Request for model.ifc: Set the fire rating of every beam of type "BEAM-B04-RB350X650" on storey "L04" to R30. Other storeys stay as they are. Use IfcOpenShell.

First a look at what the model holds.

```python
import ifcopenshell
import ifcopenshell.util.element

model = ifcopenshell.open("model.ifc")
print(model.schema)
storey = next(s for s in model.by_type("IfcBuildingStorey") if s.Name == "L04")
beams = [e for e in ifcopenshell.util.element.get_decomposition(storey) if e.is_a("IfcBeam")]
seen = {}
for e in beams:
    element_type = ifcopenshell.util.element.get_type(e)
    key = (element_type.Name if element_type != e and element_type else None, ifcopenshell.util.element.get_pset(e, "Pset_BeamCommon", "FireRating"))
    seen[key] = seen.get(key, 0) + 1
for (name, value), count in sorted(seen.items(), key=str):
    print(count, "x", name, "|", value)
```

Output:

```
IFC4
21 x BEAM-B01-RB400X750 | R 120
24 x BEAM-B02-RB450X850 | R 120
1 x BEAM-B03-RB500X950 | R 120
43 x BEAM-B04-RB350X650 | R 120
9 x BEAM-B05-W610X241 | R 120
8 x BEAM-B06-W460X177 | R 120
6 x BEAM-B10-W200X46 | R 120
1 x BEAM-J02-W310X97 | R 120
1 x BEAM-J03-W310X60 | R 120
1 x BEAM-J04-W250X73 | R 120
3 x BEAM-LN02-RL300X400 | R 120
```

```python
import ifcopenshell
import ifcopenshell.api.pset
import ifcopenshell.util.element

model = ifcopenshell.open("model.ifc")

storey = next(s for s in model.by_type("IfcBuildingStorey") if s.Name == "L04")
beams = [e for e in ifcopenshell.util.element.get_decomposition(storey) if e.is_a("IfcBeam")]

count = 0
for e in beams:
    element_type = ifcopenshell.util.element.get_type(e)
    if element_type in (None, e) or element_type.Name != "BEAM-B04-RB350X650":
        continue
    # add_pset returns the element's existing set when there is one.
    pset = ifcopenshell.api.pset.add_pset(model, product=e, name="Pset_BeamCommon")
    ifcopenshell.api.pset.edit_pset(model, pset=pset, properties={"FireRating": "R30"})
    count += 1

print(count, "beams updated")

model.write("model_rev.ifc")
```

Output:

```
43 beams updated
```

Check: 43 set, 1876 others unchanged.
